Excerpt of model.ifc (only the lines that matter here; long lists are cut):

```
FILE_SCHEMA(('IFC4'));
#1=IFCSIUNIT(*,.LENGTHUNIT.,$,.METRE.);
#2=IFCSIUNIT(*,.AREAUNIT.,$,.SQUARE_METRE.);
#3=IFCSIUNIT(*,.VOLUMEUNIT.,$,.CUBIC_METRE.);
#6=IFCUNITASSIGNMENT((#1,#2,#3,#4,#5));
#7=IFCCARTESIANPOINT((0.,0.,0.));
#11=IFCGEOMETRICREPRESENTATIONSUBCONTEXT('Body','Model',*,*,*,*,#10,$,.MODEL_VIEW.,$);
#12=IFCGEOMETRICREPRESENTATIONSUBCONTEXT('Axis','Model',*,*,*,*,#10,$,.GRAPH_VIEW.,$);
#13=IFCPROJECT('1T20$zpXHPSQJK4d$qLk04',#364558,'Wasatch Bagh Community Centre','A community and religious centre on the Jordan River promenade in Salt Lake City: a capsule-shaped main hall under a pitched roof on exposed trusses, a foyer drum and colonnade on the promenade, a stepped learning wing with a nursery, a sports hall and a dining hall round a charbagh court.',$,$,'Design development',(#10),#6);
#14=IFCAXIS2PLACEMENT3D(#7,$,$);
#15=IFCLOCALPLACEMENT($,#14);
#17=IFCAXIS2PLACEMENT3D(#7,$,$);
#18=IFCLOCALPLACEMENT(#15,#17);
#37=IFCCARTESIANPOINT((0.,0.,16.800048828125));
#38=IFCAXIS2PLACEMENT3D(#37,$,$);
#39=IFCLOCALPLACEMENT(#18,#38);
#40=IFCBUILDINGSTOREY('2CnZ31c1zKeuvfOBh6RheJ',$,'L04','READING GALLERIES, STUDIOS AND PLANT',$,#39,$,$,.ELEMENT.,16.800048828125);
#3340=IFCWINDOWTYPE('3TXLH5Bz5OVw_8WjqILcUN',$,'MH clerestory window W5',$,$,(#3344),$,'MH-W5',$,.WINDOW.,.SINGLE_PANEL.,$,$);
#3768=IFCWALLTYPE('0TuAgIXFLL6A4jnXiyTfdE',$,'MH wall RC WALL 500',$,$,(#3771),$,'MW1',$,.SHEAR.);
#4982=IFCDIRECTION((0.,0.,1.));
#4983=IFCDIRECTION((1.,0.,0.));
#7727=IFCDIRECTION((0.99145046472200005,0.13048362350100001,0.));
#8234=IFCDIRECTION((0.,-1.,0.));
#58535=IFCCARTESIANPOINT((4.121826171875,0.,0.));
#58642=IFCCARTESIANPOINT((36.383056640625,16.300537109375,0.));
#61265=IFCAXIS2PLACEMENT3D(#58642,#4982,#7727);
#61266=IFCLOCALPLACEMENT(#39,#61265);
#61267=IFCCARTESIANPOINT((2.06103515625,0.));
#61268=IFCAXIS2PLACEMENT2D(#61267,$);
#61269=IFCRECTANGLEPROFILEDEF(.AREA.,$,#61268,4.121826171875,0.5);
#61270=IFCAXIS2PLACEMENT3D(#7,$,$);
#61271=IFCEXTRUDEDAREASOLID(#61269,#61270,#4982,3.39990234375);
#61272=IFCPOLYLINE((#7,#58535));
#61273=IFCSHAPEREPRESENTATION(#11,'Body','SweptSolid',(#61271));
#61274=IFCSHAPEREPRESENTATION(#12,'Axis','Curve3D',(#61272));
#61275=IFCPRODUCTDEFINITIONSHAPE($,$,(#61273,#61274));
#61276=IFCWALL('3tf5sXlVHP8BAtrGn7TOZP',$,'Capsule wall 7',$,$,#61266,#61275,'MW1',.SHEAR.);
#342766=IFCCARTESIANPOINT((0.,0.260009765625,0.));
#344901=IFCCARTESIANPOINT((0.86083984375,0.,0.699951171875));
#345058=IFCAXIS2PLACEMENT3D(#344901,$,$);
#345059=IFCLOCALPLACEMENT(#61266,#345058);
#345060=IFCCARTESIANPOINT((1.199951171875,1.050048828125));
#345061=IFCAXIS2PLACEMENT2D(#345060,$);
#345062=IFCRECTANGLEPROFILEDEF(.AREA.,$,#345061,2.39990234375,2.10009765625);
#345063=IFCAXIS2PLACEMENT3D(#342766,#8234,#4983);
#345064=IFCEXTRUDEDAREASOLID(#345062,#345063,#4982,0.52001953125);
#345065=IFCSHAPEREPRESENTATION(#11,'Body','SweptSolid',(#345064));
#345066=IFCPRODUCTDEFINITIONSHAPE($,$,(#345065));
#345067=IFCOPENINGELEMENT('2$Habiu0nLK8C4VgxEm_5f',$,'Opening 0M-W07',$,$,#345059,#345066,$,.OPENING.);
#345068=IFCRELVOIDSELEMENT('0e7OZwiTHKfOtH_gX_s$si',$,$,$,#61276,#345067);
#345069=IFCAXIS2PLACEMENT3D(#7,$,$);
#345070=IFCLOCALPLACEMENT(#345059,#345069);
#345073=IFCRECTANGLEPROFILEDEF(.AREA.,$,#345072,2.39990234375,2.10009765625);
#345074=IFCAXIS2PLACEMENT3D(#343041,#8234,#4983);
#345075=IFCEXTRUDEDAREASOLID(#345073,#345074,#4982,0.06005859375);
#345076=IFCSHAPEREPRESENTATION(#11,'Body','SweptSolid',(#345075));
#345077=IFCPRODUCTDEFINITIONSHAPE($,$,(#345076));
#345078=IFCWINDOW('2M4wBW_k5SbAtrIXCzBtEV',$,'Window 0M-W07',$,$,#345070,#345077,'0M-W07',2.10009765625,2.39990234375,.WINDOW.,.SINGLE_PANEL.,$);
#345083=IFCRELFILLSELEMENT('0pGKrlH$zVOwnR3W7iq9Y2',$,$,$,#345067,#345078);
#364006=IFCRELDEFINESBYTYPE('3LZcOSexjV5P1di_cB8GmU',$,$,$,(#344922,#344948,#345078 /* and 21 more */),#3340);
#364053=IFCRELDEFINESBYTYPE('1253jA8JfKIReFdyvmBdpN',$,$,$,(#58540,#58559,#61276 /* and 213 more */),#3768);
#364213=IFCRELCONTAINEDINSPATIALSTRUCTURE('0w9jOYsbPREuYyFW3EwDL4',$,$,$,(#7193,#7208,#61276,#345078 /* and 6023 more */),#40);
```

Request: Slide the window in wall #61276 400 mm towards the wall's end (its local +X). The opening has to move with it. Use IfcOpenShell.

```python
import ifcopenshell
import ifcopenshell.api.geometry
import ifcopenshell.util.placement
import ifcopenshell.util.unit

model = ifcopenshell.open("model.ifc")
unit_scale = ifcopenshell.util.unit.calculate_unit_scale(model)

window = model.by_id(345078)
opening = window.FillsVoids[0].RelatingOpeningElement
wall = opening.VoidsElements[0].RelatingBuildingElement

wall_matrix = ifcopenshell.util.placement.get_local_placement(wall.ObjectPlacement)
shift = wall_matrix[:3, 0] * 0.4 / unit_scale
before = ifcopenshell.util.placement.get_local_placement(window.ObjectPlacement)[:3, 3].copy()

# The window is placed relative to its opening, so it follows when the opening moves.
matrix = ifcopenshell.util.placement.get_local_placement(opening.ObjectPlacement)
matrix[:3, 3] += shift
ifcopenshell.api.geometry.edit_object_placement(
    model, product=opening, matrix=matrix, is_si=False, should_transform_children=True
)

after = ifcopenshell.util.placement.get_local_placement(window.ObjectPlacement)[:3, 3]
print("window moved by", (after - before).round(3) + 0.0)

model.write("model_v2.ifc")
```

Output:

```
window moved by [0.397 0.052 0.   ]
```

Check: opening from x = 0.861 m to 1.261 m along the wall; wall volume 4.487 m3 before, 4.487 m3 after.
